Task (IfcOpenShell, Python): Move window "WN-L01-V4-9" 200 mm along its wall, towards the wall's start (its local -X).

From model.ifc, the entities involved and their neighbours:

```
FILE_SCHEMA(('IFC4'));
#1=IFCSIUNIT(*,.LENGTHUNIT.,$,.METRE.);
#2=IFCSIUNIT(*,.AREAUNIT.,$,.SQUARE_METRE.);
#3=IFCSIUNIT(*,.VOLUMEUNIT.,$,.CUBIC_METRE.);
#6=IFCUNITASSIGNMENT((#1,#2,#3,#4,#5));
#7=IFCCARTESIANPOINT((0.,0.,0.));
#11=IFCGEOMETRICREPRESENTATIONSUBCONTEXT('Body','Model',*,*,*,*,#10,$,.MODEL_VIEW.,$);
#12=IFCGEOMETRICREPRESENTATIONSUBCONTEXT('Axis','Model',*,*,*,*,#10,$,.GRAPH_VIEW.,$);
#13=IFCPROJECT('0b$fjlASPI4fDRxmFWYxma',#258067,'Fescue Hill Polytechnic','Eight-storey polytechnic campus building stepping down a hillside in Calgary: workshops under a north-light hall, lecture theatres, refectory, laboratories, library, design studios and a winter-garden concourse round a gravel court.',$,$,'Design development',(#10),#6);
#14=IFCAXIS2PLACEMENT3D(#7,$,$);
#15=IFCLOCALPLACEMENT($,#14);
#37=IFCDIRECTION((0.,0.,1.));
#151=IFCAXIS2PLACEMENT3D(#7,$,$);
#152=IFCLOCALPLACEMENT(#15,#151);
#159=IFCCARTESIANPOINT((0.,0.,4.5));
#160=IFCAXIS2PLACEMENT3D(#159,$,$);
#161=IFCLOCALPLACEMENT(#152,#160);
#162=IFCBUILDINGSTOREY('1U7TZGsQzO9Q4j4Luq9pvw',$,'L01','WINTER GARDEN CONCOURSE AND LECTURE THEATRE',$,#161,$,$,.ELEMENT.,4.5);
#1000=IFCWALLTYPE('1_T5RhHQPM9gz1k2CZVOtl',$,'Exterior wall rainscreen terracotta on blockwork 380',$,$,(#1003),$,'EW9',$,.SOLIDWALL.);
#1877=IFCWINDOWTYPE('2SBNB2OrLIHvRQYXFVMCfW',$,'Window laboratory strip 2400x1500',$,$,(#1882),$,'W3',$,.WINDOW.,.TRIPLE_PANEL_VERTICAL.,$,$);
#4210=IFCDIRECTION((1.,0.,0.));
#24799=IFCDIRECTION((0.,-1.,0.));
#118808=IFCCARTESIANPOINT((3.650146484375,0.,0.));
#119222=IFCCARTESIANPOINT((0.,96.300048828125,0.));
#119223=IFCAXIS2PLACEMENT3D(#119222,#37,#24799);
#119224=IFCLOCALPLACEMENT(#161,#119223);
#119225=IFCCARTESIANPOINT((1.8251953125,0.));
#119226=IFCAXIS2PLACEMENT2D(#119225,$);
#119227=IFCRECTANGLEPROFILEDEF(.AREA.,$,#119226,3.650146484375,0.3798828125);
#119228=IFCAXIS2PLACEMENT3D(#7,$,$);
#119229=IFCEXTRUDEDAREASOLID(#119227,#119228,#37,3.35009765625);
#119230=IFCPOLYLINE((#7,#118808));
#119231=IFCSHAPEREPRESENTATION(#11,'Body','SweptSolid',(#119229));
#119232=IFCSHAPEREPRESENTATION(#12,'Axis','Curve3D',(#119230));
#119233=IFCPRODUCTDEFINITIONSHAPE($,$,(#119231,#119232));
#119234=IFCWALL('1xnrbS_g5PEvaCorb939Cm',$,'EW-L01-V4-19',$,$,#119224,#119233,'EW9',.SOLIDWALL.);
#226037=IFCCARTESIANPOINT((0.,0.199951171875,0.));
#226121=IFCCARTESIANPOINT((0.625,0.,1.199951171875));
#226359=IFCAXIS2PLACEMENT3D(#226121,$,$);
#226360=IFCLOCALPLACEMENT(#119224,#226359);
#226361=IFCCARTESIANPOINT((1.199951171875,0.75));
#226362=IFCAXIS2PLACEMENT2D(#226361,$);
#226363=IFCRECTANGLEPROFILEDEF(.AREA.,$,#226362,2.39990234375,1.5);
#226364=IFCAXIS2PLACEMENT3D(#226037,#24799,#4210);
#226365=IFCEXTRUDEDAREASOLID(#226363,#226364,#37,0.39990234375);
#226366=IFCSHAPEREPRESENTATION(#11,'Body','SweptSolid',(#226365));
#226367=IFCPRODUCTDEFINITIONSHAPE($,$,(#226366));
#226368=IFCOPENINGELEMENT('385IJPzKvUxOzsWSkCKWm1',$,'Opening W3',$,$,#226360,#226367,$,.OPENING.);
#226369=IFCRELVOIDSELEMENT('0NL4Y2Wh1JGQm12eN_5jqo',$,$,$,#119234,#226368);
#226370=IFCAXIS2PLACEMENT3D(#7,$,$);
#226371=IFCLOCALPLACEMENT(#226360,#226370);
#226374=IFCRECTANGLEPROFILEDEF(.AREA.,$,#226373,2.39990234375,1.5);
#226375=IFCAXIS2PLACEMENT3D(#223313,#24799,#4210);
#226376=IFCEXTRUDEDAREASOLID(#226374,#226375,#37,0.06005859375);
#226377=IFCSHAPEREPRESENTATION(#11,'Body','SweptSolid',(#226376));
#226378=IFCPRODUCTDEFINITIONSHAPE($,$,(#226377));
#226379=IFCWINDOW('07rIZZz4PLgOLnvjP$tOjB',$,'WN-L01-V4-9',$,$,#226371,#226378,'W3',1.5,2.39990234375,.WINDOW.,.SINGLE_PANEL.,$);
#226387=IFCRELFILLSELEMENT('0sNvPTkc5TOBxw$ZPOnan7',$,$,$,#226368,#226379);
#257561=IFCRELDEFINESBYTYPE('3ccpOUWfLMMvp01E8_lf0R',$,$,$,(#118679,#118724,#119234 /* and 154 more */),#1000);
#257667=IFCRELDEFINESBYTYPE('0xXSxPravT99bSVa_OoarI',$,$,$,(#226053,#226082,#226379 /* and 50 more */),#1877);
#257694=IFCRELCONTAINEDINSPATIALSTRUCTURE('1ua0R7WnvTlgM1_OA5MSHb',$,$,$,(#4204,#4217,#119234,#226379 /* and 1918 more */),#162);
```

```python
import ifcopenshell
import ifcopenshell.api.geometry
import ifcopenshell.util.placement
import ifcopenshell.util.unit

model = ifcopenshell.open("model.ifc")
unit_scale = ifcopenshell.util.unit.calculate_unit_scale(model)

window = model.by_guid("07rIZZz4PLgOLnvjP$tOjB")
opening = window.FillsVoids[0].RelatingOpeningElement
wall = opening.VoidsElements[0].RelatingBuildingElement

wall_matrix = ifcopenshell.util.placement.get_local_placement(wall.ObjectPlacement)
shift = wall_matrix[:3, 0] * -0.2 / unit_scale
before = ifcopenshell.util.placement.get_local_placement(window.ObjectPlacement)[:3, 3].copy()

# The window is placed relative to its opening, so it follows when the opening moves.
matrix = ifcopenshell.util.placement.get_local_placement(opening.ObjectPlacement)
matrix[:3, 3] += shift
ifcopenshell.api.geometry.edit_object_placement(
    model, product=opening, matrix=matrix, is_si=False, should_transform_children=True
)

after = ifcopenshell.util.placement.get_local_placement(window.ObjectPlacement)[:3, 3]
print("window moved by", (after - before).round(3) + 0.0)

model.write("model-out.ifc")
```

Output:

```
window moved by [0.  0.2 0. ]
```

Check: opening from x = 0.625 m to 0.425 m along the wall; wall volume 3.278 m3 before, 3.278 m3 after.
